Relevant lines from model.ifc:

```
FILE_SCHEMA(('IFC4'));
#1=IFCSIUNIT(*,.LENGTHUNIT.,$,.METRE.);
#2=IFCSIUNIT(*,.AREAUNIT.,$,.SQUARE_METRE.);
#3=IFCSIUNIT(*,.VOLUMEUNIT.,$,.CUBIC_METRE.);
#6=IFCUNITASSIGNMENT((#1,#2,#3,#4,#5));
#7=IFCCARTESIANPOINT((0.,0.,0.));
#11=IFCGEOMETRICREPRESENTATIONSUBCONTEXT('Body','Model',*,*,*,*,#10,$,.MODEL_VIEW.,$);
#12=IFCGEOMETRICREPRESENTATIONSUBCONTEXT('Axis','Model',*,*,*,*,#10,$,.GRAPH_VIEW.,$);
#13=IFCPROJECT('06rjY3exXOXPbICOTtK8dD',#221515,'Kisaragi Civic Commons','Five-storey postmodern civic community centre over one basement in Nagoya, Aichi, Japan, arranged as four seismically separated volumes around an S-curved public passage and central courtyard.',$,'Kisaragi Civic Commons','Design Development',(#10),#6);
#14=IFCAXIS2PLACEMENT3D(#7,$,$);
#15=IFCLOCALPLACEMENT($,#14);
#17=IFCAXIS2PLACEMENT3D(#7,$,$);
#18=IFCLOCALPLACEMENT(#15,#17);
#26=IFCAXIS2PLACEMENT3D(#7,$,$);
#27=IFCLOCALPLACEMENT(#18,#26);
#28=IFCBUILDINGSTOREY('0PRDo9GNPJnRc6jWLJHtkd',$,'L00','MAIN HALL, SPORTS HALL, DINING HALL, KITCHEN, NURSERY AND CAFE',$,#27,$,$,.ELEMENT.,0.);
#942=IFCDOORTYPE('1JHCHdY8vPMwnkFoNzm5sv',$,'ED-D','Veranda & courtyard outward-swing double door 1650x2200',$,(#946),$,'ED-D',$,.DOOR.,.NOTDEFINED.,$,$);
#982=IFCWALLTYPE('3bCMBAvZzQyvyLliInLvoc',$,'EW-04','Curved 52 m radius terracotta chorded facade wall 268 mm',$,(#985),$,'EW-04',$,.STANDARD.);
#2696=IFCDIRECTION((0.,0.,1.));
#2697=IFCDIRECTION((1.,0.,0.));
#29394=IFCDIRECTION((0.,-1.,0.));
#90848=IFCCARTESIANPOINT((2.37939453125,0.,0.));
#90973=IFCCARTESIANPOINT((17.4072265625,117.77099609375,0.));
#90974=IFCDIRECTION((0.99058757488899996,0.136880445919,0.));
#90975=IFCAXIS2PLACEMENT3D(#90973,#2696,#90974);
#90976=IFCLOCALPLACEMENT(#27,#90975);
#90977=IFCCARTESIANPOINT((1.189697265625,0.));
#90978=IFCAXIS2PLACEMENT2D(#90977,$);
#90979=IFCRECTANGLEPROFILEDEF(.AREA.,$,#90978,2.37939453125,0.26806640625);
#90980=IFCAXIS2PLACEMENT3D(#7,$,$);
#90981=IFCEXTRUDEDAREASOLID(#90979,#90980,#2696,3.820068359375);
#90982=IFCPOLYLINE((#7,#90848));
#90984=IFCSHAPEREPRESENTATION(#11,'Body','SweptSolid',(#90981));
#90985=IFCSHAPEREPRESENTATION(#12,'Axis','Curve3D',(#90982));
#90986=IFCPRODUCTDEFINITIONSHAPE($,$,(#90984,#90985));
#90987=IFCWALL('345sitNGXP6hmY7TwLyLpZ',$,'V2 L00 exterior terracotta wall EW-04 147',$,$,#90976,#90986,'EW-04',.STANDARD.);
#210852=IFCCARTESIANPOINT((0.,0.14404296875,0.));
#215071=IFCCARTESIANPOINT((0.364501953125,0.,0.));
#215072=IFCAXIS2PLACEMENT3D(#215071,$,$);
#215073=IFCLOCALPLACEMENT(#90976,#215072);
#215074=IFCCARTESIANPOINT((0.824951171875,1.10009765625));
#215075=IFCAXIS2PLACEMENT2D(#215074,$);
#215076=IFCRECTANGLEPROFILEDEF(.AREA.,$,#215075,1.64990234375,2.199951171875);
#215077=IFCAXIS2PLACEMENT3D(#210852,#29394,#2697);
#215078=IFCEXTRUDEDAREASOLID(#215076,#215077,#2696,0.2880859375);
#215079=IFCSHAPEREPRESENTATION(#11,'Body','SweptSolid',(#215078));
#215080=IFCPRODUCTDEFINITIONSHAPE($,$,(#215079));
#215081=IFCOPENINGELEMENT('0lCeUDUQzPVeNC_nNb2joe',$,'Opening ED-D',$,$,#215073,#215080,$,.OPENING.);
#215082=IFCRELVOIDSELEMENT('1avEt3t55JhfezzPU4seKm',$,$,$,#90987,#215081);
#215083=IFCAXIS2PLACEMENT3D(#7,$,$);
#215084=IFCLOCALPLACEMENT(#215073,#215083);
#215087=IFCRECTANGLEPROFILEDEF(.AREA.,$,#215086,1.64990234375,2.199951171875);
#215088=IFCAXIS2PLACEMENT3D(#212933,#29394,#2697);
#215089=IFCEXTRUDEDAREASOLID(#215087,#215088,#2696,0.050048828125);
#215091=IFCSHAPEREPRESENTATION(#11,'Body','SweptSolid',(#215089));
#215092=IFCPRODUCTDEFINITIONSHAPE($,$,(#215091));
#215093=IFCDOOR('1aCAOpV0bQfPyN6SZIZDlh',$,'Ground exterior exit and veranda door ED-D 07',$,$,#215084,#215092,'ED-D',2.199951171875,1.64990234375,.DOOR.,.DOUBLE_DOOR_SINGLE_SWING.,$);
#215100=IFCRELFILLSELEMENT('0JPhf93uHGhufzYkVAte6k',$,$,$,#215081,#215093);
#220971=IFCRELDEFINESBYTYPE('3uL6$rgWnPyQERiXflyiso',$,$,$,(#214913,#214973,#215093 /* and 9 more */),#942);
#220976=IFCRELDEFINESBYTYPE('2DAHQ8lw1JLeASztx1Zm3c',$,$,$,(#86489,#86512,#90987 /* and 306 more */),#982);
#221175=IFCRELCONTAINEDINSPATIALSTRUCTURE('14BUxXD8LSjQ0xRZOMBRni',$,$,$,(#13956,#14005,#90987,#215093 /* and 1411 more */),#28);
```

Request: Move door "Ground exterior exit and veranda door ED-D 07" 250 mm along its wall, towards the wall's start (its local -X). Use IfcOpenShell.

```python
import ifcopenshell
import ifcopenshell.api.geometry
import ifcopenshell.util.placement
import ifcopenshell.util.unit

model = ifcopenshell.open("model.ifc")
unit_scale = ifcopenshell.util.unit.calculate_unit_scale(model)

door = model.by_guid("1aCAOpV0bQfPyN6SZIZDlh")
opening = door.FillsVoids[0].RelatingOpeningElement
wall = opening.VoidsElements[0].RelatingBuildingElement

wall_matrix = ifcopenshell.util.placement.get_local_placement(wall.ObjectPlacement)
shift = wall_matrix[:3, 0] * -0.25 / unit_scale
before = ifcopenshell.util.placement.get_local_placement(door.ObjectPlacement)[:3, 3].copy()

# The door is placed relative to its opening, so it follows when the opening moves.
matrix = ifcopenshell.util.placement.get_local_placement(opening.ObjectPlacement)
matrix[:3, 3] += shift
ifcopenshell.api.geometry.edit_object_placement(
    model, product=opening, matrix=matrix, is_si=False, should_transform_children=True
)

after = ifcopenshell.util.placement.get_local_placement(door.ObjectPlacement)[:3, 3]
print("door moved by", (after - before).round(3) + 0.0)

model.write("model_edited.ifc")
```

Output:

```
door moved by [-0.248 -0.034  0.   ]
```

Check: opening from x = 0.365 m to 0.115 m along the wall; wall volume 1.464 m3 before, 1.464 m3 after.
